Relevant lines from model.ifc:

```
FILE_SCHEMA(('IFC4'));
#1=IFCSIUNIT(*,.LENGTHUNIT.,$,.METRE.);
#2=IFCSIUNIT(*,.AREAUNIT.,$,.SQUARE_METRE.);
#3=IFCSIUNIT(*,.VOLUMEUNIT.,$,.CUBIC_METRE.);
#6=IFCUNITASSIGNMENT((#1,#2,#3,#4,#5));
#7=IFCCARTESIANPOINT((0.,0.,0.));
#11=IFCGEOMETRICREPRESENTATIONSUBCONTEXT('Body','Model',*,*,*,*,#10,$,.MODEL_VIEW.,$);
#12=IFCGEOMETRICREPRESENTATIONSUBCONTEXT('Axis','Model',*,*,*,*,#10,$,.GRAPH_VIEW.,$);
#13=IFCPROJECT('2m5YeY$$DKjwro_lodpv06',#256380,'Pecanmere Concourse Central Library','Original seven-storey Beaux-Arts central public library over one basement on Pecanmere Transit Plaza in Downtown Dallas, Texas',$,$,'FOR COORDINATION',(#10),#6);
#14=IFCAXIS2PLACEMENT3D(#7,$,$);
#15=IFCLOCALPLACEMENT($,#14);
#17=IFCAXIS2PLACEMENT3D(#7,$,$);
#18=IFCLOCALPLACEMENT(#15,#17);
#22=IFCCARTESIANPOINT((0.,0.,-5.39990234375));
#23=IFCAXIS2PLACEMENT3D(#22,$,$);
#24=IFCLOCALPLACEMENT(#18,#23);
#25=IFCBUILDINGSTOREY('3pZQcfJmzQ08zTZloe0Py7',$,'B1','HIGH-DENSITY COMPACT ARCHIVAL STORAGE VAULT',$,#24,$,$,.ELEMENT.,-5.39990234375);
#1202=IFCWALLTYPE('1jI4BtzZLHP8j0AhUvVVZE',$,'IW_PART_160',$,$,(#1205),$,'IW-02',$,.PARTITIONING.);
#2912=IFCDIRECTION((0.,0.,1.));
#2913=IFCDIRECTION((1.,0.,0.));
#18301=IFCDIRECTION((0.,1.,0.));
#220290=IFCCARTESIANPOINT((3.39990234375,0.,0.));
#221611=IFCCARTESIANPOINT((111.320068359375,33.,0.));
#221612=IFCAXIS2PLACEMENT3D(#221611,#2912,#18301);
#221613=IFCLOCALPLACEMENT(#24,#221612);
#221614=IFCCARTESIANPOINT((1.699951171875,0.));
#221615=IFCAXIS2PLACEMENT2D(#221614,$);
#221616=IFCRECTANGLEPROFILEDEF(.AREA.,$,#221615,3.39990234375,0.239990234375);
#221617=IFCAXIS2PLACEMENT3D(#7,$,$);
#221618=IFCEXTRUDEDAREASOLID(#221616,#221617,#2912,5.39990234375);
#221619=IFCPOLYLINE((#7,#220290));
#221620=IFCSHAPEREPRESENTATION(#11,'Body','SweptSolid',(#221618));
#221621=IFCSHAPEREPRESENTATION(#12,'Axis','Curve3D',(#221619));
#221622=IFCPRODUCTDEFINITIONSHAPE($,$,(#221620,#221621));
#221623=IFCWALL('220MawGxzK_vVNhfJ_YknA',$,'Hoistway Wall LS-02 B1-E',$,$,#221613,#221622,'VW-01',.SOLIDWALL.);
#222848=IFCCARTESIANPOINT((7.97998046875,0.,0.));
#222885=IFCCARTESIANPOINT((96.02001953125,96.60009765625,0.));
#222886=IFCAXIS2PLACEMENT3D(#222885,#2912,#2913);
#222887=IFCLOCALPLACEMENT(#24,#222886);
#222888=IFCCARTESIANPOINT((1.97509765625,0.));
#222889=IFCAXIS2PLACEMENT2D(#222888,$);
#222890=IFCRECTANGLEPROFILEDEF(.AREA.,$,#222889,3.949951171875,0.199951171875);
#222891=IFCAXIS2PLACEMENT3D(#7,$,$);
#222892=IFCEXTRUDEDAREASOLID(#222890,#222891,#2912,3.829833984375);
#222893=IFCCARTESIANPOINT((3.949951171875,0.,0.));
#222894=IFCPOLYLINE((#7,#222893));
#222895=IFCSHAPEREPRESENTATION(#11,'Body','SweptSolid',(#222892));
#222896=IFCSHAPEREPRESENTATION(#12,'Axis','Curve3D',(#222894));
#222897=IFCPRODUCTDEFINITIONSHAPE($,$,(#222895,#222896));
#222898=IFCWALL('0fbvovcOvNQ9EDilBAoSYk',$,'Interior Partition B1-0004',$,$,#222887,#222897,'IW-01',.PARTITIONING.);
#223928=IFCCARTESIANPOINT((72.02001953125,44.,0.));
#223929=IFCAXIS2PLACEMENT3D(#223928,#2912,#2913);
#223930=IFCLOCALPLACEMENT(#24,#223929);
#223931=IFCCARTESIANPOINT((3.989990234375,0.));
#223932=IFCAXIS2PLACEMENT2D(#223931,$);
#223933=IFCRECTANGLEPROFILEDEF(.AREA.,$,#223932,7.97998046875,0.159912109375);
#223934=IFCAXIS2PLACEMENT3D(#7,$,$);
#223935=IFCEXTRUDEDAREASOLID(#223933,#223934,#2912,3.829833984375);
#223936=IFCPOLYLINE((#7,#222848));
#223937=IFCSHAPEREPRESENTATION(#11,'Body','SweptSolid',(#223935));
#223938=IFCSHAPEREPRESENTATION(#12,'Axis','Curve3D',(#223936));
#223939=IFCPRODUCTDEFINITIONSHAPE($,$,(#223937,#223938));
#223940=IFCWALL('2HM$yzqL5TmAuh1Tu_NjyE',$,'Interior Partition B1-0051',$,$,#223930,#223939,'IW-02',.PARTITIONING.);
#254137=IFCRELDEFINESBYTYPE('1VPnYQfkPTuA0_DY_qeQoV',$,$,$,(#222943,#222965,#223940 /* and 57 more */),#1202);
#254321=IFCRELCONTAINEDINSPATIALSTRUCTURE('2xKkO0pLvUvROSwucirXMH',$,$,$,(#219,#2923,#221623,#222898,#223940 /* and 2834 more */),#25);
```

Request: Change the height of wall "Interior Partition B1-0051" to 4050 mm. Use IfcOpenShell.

```python
import ifcopenshell
import ifcopenshell.geom
import ifcopenshell.util.representation
import ifcopenshell.util.shape

model = ifcopenshell.open("model.ifc")
settings = ifcopenshell.geom.settings()


def volume(element):
    """Net volume in cubic metres, openings subtracted."""
    shape = ifcopenshell.geom.create_shape(settings, element)
    return ifcopenshell.util.shape.get_volume(shape.geometry)


wall = model.by_id(223940)
before = volume(wall)

body = ifcopenshell.util.representation.get_representation(wall, "Model", "Body")
solid = body.Items[0]
old_height = solid.Depth
solid.Depth = 4.05
after = volume(wall)

print(f"height {old_height:g} -> {solid.Depth:g}, volume {before:.3f} -> {after:.3f} m3")

model.write("model_rev.ifc")
```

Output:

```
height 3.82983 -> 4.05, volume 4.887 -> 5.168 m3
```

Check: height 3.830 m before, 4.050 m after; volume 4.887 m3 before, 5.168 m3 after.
